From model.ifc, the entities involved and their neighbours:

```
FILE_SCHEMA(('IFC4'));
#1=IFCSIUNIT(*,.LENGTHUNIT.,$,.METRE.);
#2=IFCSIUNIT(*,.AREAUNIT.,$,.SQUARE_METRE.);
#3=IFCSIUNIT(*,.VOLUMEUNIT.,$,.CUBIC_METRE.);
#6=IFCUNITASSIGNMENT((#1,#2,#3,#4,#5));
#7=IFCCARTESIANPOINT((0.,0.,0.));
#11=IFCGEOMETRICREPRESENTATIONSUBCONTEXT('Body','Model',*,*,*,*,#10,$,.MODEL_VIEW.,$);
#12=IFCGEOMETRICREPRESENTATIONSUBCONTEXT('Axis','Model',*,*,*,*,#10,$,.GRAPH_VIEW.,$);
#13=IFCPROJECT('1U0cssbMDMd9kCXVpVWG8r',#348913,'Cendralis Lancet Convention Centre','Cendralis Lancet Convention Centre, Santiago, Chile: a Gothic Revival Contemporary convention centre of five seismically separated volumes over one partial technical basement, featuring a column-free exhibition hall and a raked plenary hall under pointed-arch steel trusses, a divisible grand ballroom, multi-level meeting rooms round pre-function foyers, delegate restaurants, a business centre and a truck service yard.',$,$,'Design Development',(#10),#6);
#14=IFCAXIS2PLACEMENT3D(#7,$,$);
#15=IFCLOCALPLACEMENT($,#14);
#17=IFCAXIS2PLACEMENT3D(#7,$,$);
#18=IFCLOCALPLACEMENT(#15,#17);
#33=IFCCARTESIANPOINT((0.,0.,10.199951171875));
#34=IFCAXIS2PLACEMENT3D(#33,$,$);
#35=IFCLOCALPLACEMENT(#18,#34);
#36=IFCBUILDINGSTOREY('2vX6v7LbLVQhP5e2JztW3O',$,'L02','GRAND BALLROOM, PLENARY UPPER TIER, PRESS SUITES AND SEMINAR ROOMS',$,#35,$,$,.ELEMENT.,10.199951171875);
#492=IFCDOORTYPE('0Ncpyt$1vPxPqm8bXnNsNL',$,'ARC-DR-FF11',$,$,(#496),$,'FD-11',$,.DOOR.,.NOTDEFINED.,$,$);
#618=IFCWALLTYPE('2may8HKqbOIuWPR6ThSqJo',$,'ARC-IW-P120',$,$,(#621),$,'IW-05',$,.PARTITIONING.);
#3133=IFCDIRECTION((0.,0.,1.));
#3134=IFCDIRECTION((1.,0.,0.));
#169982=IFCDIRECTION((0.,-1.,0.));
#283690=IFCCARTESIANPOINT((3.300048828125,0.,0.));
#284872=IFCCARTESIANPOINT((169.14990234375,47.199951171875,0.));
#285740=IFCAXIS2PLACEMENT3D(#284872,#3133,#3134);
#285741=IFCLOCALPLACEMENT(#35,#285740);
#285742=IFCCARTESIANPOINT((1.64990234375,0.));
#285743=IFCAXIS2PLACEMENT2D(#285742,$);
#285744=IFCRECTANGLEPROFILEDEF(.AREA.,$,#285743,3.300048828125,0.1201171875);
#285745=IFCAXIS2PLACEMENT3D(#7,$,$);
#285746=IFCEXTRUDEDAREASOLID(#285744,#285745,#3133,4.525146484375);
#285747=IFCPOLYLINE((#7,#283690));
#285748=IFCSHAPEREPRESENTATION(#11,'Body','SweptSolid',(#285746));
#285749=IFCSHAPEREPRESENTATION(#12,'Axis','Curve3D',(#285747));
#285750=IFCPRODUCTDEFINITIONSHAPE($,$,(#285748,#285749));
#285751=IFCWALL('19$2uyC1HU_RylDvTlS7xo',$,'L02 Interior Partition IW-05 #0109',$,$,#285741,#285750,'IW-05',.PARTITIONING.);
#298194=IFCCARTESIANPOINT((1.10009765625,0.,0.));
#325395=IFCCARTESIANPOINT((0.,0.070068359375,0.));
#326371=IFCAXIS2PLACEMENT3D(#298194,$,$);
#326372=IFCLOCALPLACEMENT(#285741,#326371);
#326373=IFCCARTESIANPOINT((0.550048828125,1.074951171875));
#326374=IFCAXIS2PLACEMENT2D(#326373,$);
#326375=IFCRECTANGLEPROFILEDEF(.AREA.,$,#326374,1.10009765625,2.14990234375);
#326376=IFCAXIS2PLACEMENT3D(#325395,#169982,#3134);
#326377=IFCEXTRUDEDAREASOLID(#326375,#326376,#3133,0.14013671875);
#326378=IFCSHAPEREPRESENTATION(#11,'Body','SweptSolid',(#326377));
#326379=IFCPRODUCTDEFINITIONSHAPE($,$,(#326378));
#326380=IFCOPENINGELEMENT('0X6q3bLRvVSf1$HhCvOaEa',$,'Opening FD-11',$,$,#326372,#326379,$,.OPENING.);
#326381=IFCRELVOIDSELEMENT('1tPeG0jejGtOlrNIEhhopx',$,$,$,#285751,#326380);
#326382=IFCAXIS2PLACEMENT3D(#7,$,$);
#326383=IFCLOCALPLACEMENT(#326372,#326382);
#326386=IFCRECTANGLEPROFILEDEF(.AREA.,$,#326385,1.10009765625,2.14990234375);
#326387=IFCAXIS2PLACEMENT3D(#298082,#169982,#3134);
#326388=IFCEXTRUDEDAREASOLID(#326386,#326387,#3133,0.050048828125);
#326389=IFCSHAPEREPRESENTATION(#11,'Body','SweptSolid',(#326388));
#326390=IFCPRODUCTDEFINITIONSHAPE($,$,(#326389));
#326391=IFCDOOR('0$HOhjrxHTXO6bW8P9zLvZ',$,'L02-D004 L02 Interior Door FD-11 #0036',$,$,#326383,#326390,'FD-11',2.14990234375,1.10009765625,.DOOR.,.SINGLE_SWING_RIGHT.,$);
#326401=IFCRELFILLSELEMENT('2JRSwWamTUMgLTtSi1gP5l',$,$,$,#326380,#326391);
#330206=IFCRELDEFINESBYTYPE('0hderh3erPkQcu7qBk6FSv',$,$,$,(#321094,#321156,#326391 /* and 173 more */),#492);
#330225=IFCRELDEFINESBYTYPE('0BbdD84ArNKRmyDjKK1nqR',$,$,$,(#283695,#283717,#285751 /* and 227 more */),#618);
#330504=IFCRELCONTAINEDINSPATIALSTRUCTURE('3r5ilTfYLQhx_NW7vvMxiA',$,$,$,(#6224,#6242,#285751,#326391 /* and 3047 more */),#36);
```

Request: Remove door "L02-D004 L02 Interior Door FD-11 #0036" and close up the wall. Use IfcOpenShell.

```python
import ifcopenshell
import ifcopenshell.api.feature
import ifcopenshell.api.root
import ifcopenshell.geom
import ifcopenshell.util.shape

model = ifcopenshell.open("model.ifc")
settings = ifcopenshell.geom.settings()


def volume(element):
    """Net volume in cubic metres, openings subtracted."""
    shape = ifcopenshell.geom.create_shape(settings, element)
    return ifcopenshell.util.shape.get_volume(shape.geometry)


door = model.by_guid("0$HOhjrxHTXO6bW8P9zLvZ")
opening = door.FillsVoids[0].RelatingOpeningElement
wall = opening.VoidsElements[0].RelatingBuildingElement
before = volume(wall)

ifcopenshell.api.root.remove_product(model, product=door)
ifcopenshell.api.feature.remove_feature(model, feature=opening)

after = volume(wall)

print(f"wall volume {before:.3f} -> {after:.3f} m3")

model.write("model-out.ifc")
```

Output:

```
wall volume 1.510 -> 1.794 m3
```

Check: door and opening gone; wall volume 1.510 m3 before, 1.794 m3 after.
